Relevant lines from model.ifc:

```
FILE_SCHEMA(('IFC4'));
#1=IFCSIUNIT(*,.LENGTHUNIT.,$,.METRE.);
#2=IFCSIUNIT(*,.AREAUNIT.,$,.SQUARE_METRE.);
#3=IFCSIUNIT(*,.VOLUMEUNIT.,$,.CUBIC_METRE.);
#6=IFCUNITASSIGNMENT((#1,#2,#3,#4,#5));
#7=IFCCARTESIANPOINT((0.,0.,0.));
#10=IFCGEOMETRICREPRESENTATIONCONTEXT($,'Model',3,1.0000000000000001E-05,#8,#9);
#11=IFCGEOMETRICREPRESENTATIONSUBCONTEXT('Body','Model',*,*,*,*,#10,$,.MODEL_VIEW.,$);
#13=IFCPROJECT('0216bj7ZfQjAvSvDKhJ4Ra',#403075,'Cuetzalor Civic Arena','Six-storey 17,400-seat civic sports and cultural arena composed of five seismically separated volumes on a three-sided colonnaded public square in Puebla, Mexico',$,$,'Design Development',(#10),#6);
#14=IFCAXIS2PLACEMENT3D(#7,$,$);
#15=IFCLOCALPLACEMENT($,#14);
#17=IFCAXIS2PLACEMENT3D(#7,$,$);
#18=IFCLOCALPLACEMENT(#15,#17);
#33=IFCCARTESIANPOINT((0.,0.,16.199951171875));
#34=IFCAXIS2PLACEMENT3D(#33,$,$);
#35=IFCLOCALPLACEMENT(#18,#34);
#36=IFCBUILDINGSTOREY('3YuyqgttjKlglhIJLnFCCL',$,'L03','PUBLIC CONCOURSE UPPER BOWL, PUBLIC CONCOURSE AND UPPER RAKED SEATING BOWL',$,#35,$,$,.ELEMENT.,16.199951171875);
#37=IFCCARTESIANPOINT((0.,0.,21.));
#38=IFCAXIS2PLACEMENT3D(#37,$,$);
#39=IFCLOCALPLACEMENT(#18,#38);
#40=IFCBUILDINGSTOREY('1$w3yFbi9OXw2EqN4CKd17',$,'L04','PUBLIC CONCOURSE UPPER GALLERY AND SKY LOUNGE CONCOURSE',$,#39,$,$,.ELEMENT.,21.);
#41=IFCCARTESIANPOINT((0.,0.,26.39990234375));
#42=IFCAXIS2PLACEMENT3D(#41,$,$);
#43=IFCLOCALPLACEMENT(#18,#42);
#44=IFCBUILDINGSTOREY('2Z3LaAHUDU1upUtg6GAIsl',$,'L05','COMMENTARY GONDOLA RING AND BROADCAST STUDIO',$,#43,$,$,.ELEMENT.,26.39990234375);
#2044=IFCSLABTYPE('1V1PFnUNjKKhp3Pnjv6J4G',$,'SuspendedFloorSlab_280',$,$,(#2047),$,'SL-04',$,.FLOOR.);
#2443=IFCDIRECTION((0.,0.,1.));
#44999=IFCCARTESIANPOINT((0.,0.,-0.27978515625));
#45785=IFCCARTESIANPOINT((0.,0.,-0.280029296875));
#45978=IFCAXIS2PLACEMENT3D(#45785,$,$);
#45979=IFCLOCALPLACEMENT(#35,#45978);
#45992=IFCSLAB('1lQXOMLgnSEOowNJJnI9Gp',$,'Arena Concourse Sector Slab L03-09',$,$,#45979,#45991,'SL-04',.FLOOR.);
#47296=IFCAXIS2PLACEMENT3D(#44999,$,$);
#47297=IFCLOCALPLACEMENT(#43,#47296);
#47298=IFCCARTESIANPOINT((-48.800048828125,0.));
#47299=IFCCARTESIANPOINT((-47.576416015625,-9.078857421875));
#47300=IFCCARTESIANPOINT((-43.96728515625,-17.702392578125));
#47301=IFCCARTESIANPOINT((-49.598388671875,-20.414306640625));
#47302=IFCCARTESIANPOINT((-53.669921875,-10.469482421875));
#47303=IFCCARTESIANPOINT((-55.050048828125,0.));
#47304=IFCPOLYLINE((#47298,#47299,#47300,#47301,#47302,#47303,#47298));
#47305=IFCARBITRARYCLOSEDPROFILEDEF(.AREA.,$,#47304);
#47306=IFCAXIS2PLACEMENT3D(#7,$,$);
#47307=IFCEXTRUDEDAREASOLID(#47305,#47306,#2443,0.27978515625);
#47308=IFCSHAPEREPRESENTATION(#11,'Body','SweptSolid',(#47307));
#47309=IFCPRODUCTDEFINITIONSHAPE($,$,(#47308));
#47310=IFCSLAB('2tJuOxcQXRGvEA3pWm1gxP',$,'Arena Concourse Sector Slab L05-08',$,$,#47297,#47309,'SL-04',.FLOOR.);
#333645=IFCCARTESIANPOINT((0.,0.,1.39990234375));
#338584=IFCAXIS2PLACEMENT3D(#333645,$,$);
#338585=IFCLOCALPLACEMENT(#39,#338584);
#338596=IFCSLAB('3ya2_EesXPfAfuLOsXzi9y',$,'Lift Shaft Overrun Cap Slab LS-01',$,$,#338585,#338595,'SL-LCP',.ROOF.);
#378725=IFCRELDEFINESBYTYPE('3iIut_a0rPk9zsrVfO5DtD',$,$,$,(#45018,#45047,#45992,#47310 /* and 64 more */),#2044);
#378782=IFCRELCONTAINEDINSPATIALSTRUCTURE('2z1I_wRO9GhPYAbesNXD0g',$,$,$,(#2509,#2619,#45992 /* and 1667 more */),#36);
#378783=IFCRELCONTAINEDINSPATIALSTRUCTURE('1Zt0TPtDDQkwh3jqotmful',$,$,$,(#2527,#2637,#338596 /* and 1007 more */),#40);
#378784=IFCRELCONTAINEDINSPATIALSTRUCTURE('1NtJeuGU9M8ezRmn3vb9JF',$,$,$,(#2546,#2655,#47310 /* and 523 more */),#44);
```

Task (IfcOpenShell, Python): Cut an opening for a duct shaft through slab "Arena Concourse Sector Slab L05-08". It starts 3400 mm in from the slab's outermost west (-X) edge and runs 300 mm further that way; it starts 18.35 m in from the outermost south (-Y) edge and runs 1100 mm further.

```python
import numpy as np
import ifcopenshell
import ifcopenshell.api.feature
import ifcopenshell.api.geometry
import ifcopenshell.api.root
import ifcopenshell.geom
import ifcopenshell.util.placement
import ifcopenshell.util.representation
import ifcopenshell.util.shape
import ifcopenshell.util.unit

model = ifcopenshell.open("model.ifc")
unit_scale = ifcopenshell.util.unit.calculate_unit_scale(model)
settings = ifcopenshell.geom.settings()


def volume(element):
    """Net volume in cubic metres, openings subtracted."""
    shape = ifcopenshell.geom.create_shape(settings, element)
    return ifcopenshell.util.shape.get_volume(shape.geometry)


slab = model.by_guid("2tJuOxcQXRGvEA3pWm1gxP")
before = volume(slab)

# Extent in the slab's own axes, in metres. The edges named are its -X and -Y sides.
slab_shape = ifcopenshell.geom.create_shape(settings, slab)
vertices = ifcopenshell.util.shape.get_vertices(slab_shape.geometry)
x_min, y_min, bottom = vertices.min(axis=0)
top = vertices[:, 2].max()

opening = ifcopenshell.api.root.create_entity(model, ifc_class="IfcOpeningElement", name="Duct shaft opening", predefined_type="OPENING")
context = ifcopenshell.util.representation.get_context(model, "Model", "Body", "MODEL_VIEW")
width, depth = 0.3, 1.1
outline = [(0.0, 0.0), (width, 0.0), (width, depth), (0.0, depth), (0.0, 0.0)]
# Overshoot both faces by 50 mm so the cut is clean.
shape = ifcopenshell.api.geometry.add_slab_representation(
    model, context=context, depth=top - bottom + 0.1, polyline=outline
)
ifcopenshell.api.geometry.assign_representation(model, product=opening, representation=shape)

matrix = ifcopenshell.util.placement.get_local_placement(slab.ObjectPlacement)
matrix[:, 3] = matrix @ np.append(np.array([x_min + 3.4, y_min + 18.35, bottom - 0.05]) / unit_scale, 1.0)
ifcopenshell.api.geometry.edit_object_placement(model, product=opening, matrix=matrix, is_si=False)
ifcopenshell.api.feature.add_feature(model, feature=opening, element=slab)

after = volume(slab)

print(f"slab volume {before:.3f} -> {after:.3f} m3")

model.write("model-out.ifc")
```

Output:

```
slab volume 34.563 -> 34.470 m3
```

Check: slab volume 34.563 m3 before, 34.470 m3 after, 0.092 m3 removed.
